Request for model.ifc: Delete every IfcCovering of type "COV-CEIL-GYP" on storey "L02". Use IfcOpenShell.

First a look at what the model holds.

```python
import ifcopenshell
import ifcopenshell.util.element

model = ifcopenshell.open("model.ifc")
print(model.schema)
storey = next(s for s in model.by_type("IfcBuildingStorey") if s.Name == "L02")
coverings = [e for e in ifcopenshell.util.element.get_decomposition(storey) if e.is_a("IfcCovering")]
seen = {}
for e in coverings:
    element_type = ifcopenshell.util.element.get_type(e)
    name = element_type.Name if element_type not in (None, e) else None
    seen[name] = seen.get(name, 0) + 1
for name, count in sorted(seen.items(), key=str):
    print(count, "x", name)
```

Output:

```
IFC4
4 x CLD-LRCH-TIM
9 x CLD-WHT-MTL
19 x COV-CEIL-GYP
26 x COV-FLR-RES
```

```python
import ifcopenshell
import ifcopenshell.api.root
import ifcopenshell.util.element

model = ifcopenshell.open("model.ifc")

storey = next(s for s in model.by_type("IfcBuildingStorey") if s.Name == "L02")
coverings = [e for e in ifcopenshell.util.element.get_decomposition(storey) if e.is_a("IfcCovering")]
targets = [e for e in coverings if (t := ifcopenshell.util.element.get_type(e)) not in (None, e) and t.Name == "COV-CEIL-GYP"]

for e in targets:
    ifcopenshell.api.root.remove_product(model, product=e)
print(len(targets), "removed")

model.write("model_v2.ifc")
```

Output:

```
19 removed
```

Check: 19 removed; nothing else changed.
